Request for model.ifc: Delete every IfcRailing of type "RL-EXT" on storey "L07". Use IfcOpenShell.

First a look at what the model holds.

```python
import ifcopenshell
import ifcopenshell.util.element

model = ifcopenshell.open("model.ifc")
print(model.schema)
storey = next(s for s in model.by_type("IfcBuildingStorey") if s.Name == "L07")
railings = [e for e in ifcopenshell.util.element.get_decomposition(storey) if e.is_a("IfcRailing")]
seen = {}
for e in railings:
    element_type = ifcopenshell.util.element.get_type(e)
    name = element_type.Name if element_type not in (None, e) else None
    seen[name] = seen.get(name, 0) + 1
for name, count in sorted(seen.items(), key=str):
    print(count, "x", name)
```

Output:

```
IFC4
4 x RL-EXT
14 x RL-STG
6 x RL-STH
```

```python
import ifcopenshell
import ifcopenshell.api.root
import ifcopenshell.util.element

model = ifcopenshell.open("model.ifc")

storey = next(s for s in model.by_type("IfcBuildingStorey") if s.Name == "L07")
railings = [e for e in ifcopenshell.util.element.get_decomposition(storey) if e.is_a("IfcRailing")]
targets = [e for e in railings if (t := ifcopenshell.util.element.get_type(e)) not in (None, e) and t.Name == "RL-EXT"]

for e in targets:
    ifcopenshell.api.root.remove_product(model, product=e)
print(len(targets), "removed")

model.write("model_v2.ifc")
```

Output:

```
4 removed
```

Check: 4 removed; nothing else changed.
